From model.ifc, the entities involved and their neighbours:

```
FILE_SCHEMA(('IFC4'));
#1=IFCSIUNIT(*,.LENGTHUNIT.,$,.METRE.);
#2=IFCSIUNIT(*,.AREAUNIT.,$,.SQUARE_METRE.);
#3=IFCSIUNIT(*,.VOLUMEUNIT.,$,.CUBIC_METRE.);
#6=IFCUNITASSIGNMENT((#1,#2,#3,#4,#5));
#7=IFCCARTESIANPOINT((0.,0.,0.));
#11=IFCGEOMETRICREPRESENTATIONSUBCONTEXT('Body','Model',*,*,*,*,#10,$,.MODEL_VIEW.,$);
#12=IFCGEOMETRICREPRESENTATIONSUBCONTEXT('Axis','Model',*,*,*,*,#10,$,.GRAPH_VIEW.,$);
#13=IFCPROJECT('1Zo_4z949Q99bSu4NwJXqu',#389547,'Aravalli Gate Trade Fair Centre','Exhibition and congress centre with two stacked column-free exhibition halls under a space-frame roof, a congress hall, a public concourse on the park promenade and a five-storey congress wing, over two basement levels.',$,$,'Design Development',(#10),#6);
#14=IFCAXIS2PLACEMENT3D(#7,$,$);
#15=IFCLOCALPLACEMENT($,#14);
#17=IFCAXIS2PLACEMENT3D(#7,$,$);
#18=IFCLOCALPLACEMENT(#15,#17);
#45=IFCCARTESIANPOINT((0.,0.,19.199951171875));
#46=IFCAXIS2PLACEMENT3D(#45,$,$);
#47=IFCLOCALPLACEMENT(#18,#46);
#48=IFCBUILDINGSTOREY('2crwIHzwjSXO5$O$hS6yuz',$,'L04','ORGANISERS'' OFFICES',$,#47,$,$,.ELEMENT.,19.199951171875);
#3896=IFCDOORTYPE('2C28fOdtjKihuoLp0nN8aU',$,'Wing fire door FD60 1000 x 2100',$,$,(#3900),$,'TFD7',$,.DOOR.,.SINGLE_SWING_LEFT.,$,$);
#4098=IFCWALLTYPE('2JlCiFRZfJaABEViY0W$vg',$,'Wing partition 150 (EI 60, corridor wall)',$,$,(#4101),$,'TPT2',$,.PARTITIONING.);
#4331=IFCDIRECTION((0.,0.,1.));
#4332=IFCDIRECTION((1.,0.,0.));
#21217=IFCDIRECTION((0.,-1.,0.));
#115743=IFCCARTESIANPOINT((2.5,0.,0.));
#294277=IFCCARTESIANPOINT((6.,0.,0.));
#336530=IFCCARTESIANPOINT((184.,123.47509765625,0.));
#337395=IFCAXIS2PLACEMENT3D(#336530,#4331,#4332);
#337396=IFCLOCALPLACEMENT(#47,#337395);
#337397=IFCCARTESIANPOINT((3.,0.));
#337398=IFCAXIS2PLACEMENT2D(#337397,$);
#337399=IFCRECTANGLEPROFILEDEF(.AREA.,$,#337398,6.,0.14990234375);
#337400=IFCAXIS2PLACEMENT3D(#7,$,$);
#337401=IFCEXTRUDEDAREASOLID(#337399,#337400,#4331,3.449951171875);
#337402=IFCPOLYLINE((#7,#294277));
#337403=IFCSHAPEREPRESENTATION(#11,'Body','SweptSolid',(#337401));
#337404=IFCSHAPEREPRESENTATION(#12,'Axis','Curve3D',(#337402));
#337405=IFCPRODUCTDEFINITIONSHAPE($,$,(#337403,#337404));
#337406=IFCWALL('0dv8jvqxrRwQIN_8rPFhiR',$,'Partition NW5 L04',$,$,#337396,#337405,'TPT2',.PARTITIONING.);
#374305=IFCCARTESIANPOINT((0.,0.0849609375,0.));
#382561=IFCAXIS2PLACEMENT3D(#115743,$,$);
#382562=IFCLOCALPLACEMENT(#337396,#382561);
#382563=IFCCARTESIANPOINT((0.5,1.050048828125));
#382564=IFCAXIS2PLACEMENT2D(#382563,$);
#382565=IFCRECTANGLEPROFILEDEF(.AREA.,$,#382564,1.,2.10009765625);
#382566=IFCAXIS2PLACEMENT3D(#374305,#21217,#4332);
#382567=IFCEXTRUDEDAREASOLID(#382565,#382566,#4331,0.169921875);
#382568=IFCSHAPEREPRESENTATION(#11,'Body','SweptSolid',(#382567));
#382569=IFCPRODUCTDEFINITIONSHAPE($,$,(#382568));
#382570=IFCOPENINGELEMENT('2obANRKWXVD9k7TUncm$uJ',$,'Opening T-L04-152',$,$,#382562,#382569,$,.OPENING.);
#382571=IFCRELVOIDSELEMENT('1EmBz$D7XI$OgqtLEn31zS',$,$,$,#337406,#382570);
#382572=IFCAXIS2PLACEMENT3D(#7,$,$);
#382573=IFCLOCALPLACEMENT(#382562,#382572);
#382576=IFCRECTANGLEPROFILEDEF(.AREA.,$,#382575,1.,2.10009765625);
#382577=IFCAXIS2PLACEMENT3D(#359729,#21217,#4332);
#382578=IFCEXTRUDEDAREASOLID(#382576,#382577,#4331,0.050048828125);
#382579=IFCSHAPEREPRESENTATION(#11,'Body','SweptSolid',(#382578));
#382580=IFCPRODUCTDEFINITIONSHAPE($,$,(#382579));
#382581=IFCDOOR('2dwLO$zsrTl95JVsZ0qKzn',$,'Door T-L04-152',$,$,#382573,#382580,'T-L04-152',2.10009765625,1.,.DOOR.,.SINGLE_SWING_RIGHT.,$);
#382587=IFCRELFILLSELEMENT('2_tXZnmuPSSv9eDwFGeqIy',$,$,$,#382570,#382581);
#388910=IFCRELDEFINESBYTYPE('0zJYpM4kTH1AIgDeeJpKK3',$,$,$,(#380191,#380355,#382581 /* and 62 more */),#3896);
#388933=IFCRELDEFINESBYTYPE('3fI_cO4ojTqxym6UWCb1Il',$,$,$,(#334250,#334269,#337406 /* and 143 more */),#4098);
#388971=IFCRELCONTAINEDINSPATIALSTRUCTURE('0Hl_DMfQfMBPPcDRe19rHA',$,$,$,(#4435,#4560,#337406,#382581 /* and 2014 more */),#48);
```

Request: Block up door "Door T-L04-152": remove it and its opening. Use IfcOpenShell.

```python
import ifcopenshell
import ifcopenshell.api.feature
import ifcopenshell.api.root
import ifcopenshell.geom
import ifcopenshell.util.shape

model = ifcopenshell.open("model.ifc")
settings = ifcopenshell.geom.settings()


def volume(element):
    """Net volume in cubic metres, openings subtracted."""
    shape = ifcopenshell.geom.create_shape(settings, element)
    return ifcopenshell.util.shape.get_volume(shape.geometry)


door = model.by_guid("2dwLO$zsrTl95JVsZ0qKzn")
opening = door.FillsVoids[0].RelatingOpeningElement
wall = opening.VoidsElements[0].RelatingBuildingElement
before = volume(wall)

ifcopenshell.api.root.remove_product(model, product=door)
ifcopenshell.api.feature.remove_feature(model, feature=opening)

after = volume(wall)

print(f"wall volume {before:.3f} -> {after:.3f} m3")

model.write("model_rev.ifc")
```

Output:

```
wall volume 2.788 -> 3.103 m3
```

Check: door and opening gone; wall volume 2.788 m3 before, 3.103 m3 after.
